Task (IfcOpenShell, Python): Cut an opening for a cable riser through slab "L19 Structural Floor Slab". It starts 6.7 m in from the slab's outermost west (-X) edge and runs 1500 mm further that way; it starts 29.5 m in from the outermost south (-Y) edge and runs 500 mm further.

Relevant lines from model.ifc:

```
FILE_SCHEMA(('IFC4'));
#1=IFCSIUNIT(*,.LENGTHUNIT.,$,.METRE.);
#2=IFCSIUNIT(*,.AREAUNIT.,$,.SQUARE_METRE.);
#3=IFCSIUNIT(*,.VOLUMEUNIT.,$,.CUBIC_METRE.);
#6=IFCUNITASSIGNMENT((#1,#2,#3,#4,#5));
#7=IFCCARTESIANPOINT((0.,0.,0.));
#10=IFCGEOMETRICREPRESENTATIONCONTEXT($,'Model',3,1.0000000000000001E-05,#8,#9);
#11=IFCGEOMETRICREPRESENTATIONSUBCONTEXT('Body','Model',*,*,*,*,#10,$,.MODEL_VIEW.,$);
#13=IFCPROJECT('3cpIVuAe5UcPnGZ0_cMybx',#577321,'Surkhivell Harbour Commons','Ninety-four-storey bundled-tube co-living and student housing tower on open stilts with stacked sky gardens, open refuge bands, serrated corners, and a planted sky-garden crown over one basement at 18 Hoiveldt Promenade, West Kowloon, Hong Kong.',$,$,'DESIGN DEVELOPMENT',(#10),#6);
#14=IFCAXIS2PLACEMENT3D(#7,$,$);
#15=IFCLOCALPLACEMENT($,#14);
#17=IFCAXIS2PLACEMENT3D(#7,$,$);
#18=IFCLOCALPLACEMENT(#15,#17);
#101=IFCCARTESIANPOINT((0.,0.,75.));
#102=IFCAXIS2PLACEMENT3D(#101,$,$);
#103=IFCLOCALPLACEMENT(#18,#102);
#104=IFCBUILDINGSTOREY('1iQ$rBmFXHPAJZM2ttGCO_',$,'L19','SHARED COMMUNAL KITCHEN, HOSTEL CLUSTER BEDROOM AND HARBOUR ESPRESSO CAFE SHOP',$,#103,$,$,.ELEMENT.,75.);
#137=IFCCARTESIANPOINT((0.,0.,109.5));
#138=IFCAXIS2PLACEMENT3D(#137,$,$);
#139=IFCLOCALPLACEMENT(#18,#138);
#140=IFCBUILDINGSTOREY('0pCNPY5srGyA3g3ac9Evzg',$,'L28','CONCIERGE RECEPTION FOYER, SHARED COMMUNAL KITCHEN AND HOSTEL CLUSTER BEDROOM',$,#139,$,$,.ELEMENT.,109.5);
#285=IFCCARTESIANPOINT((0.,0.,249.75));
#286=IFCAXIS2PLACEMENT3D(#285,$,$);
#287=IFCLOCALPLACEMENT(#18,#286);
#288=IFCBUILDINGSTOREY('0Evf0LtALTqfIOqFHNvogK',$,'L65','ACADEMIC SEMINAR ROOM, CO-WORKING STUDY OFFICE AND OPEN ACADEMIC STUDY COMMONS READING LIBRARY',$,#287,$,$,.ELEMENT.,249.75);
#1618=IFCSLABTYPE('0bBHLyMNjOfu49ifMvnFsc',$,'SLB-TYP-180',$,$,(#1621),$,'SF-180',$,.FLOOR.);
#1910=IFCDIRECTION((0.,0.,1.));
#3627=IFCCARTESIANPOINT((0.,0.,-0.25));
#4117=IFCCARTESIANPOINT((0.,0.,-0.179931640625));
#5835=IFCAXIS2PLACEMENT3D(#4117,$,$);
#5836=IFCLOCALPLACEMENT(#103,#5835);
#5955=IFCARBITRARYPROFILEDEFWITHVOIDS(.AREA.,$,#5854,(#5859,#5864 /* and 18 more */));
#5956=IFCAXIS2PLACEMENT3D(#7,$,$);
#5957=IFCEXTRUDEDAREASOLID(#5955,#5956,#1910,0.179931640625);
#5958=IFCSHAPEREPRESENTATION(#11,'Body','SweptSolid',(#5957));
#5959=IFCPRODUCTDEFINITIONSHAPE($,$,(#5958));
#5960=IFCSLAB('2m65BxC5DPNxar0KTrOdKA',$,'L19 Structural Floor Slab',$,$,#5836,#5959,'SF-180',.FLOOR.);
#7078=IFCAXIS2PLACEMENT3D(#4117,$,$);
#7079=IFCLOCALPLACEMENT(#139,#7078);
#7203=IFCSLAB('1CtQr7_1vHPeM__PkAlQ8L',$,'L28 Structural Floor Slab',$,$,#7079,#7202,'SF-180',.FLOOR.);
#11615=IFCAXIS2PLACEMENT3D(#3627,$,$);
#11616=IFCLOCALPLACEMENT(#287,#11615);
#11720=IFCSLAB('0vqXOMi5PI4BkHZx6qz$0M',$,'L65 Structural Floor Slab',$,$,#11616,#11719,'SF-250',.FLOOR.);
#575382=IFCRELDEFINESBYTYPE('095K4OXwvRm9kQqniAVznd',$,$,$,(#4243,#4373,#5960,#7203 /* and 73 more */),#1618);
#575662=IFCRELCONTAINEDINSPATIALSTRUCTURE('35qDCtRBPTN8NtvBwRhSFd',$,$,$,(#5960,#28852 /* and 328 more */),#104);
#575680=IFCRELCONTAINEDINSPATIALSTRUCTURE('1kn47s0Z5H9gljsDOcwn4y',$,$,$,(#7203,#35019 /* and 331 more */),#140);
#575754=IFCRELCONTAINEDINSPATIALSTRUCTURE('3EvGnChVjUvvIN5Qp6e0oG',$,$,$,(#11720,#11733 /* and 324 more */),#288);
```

```python
import numpy as np
import ifcopenshell
import ifcopenshell.api.feature
import ifcopenshell.api.geometry
import ifcopenshell.api.root
import ifcopenshell.geom
import ifcopenshell.util.placement
import ifcopenshell.util.representation
import ifcopenshell.util.shape
import ifcopenshell.util.unit

model = ifcopenshell.open("model.ifc")
unit_scale = ifcopenshell.util.unit.calculate_unit_scale(model)
settings = ifcopenshell.geom.settings()


def volume(element):
    """Net volume in cubic metres, openings subtracted."""
    shape = ifcopenshell.geom.create_shape(settings, element)
    return ifcopenshell.util.shape.get_volume(shape.geometry)


slab = model.by_guid("2m65BxC5DPNxar0KTrOdKA")
before = volume(slab)

# Extent in the slab's own axes, in metres. The edges named are its -X and -Y sides.
slab_shape = ifcopenshell.geom.create_shape(settings, slab)
vertices = ifcopenshell.util.shape.get_vertices(slab_shape.geometry)
x_min, y_min, bottom = vertices.min(axis=0)
top = vertices[:, 2].max()

opening = ifcopenshell.api.root.create_entity(model, ifc_class="IfcOpeningElement", name="Cable riser opening", predefined_type="OPENING")
context = ifcopenshell.util.representation.get_context(model, "Model", "Body", "MODEL_VIEW")
width, depth = 1.5, 0.5
outline = [(0.0, 0.0), (width, 0.0), (width, depth), (0.0, depth), (0.0, 0.0)]
# Overshoot both faces by 50 mm so the cut is clean.
shape = ifcopenshell.api.geometry.add_slab_representation(
    model, context=context, depth=top - bottom + 0.1, polyline=outline
)
ifcopenshell.api.geometry.assign_representation(model, product=opening, representation=shape)

matrix = ifcopenshell.util.placement.get_local_placement(slab.ObjectPlacement)
matrix[:, 3] = matrix @ np.append(np.array([x_min + 6.7, y_min + 29.5, bottom - 0.05]) / unit_scale, 1.0)
ifcopenshell.api.geometry.edit_object_placement(model, product=opening, matrix=matrix, is_si=False)
ifcopenshell.api.feature.add_feature(model, feature=opening, element=slab)

after = volume(slab)

print(f"slab volume {before:.3f} -> {after:.3f} m3")

model.write("model_updated.ifc")
```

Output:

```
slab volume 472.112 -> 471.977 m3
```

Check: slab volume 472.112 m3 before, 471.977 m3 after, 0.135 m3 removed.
